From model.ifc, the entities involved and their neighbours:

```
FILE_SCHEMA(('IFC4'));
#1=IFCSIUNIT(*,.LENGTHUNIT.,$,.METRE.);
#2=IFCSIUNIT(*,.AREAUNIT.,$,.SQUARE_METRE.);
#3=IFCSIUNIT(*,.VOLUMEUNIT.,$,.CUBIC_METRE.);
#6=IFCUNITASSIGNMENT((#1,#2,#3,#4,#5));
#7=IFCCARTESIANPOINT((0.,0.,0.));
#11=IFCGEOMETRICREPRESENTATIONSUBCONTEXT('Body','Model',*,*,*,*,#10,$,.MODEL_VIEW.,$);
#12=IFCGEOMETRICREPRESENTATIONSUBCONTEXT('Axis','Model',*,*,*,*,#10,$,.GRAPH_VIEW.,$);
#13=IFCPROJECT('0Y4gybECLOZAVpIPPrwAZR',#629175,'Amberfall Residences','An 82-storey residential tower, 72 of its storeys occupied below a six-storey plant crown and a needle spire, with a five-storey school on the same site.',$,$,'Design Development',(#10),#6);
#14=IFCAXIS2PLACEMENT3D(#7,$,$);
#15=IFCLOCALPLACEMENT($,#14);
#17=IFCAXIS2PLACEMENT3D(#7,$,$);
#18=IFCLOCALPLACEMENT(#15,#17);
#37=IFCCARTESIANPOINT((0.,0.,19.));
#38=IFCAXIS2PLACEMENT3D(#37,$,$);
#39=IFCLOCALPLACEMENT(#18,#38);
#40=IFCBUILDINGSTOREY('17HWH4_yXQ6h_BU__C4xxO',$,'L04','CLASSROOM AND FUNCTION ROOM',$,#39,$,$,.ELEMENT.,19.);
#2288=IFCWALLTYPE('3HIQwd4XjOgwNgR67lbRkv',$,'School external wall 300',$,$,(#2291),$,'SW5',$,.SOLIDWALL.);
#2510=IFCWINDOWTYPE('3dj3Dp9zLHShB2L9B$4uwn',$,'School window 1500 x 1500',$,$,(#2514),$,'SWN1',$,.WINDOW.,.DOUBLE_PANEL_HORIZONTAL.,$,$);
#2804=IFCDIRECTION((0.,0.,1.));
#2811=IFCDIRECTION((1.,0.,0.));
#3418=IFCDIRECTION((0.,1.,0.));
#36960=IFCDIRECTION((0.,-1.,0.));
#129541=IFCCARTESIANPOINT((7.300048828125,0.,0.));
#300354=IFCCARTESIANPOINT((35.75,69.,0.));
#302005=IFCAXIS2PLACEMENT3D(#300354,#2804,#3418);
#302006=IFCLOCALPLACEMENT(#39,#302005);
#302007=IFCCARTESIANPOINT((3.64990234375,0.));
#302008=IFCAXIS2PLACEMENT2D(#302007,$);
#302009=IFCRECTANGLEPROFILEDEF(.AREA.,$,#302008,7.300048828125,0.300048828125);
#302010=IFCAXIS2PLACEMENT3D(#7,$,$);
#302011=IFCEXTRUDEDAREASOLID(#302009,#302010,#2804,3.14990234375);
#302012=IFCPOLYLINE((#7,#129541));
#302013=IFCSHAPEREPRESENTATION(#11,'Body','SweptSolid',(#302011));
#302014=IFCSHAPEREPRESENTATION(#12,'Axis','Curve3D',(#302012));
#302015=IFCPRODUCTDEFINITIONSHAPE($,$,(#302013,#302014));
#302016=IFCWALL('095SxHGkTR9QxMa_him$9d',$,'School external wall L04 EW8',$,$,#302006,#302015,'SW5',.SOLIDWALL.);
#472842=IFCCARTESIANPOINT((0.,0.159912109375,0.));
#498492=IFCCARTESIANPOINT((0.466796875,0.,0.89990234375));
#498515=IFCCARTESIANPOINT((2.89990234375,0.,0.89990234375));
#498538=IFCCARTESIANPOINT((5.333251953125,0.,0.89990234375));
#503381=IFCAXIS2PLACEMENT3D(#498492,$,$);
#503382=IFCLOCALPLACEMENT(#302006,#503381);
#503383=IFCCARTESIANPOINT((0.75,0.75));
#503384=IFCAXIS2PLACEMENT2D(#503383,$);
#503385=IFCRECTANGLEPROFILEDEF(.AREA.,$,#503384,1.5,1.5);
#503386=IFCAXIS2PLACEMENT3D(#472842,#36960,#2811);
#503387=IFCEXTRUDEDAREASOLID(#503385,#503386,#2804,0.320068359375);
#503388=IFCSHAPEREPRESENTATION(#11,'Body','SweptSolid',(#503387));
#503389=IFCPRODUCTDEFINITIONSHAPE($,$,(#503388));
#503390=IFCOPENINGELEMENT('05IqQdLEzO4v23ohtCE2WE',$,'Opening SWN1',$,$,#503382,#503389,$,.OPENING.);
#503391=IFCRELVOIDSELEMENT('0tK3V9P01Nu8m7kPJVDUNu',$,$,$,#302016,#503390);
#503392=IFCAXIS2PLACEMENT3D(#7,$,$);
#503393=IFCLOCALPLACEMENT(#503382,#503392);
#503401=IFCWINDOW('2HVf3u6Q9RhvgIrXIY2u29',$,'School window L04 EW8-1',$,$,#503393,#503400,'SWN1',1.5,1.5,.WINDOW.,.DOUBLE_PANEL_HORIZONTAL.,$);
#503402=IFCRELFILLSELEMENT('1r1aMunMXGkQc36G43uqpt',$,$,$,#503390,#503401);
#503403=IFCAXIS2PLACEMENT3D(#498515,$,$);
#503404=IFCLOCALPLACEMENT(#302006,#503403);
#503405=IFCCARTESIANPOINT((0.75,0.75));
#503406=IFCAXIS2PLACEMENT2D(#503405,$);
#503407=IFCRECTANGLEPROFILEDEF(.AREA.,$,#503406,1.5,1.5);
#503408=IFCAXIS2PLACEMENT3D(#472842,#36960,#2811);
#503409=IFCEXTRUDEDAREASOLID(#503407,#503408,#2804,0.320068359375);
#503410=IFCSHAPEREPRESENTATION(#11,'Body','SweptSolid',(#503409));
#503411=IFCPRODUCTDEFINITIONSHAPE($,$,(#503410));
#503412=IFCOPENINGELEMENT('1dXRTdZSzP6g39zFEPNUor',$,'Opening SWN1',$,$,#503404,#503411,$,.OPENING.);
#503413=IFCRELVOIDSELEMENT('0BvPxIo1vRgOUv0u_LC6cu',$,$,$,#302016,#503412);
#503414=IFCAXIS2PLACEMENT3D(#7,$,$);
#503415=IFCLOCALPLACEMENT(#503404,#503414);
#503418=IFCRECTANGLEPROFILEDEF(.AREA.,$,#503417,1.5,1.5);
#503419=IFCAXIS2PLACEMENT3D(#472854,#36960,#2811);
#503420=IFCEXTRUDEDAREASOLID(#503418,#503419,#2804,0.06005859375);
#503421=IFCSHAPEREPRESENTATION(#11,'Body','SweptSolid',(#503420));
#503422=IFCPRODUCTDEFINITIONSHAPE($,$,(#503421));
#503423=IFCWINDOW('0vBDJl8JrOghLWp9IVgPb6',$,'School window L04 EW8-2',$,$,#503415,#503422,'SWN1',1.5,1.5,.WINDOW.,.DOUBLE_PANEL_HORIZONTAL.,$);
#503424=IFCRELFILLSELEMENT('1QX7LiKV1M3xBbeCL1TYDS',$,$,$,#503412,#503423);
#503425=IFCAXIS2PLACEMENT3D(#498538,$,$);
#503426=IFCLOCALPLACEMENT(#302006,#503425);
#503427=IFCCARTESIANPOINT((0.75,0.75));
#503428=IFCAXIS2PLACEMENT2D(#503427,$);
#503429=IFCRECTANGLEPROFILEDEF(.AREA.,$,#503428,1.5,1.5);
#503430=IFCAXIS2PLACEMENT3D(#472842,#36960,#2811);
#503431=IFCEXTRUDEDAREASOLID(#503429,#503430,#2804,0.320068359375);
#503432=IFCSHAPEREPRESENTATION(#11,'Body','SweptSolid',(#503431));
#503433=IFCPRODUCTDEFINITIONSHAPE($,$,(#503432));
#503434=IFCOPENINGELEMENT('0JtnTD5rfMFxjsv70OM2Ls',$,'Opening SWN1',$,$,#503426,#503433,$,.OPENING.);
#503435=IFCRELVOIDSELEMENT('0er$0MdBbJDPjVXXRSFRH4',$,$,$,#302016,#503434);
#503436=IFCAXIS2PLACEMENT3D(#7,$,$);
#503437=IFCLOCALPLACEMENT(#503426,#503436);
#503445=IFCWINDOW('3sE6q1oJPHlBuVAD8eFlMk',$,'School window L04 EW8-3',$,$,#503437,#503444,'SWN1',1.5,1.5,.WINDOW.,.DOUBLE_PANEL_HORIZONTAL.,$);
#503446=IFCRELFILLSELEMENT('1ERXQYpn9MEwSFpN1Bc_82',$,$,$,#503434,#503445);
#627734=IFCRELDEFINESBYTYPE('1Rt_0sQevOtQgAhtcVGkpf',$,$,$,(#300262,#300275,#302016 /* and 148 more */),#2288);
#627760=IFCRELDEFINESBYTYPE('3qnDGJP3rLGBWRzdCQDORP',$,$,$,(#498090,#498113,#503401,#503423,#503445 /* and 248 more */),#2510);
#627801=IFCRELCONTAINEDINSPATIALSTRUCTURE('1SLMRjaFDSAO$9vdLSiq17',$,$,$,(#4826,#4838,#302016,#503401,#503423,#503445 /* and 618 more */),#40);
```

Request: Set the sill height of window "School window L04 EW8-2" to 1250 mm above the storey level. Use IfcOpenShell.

```python
import numpy as np
import ifcopenshell
import ifcopenshell.api.geometry
import ifcopenshell.geom
import ifcopenshell.util.element
import ifcopenshell.util.placement
import ifcopenshell.util.shape
import ifcopenshell.util.unit

model = ifcopenshell.open("model.ifc")
unit_scale = ifcopenshell.util.unit.calculate_unit_scale(model)

window = model.by_id(503423)
opening = window.FillsVoids[0].RelatingOpeningElement
storey = ifcopenshell.util.element.get_container(window, ifc_class="IfcBuildingStorey")
level = ifcopenshell.util.placement.get_local_placement(storey.ObjectPlacement)[2, 3]

# The opening's origin need not be at the sill, so measure its lowest point.
shape = ifcopenshell.geom.create_shape(ifcopenshell.geom.settings(), opening)
bottom = ifcopenshell.util.shape.get_shape_bottom_elevation(shape, shape.geometry) / unit_scale
dz = level + 1.25 / unit_scale - bottom

shift = np.array([0.0, 0.0, dz])
# The window is placed relative to its opening, so it follows when the opening moves.
matrix = ifcopenshell.util.placement.get_local_placement(opening.ObjectPlacement)
matrix[:3, 3] += shift
ifcopenshell.api.geometry.edit_object_placement(
    model, product=opening, matrix=matrix, is_si=False, should_transform_children=True
)

print(f"moved by {dz * unit_scale:+.3f} m")

model.write("model_edited.ifc")
```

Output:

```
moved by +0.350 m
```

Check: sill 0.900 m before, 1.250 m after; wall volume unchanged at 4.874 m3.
